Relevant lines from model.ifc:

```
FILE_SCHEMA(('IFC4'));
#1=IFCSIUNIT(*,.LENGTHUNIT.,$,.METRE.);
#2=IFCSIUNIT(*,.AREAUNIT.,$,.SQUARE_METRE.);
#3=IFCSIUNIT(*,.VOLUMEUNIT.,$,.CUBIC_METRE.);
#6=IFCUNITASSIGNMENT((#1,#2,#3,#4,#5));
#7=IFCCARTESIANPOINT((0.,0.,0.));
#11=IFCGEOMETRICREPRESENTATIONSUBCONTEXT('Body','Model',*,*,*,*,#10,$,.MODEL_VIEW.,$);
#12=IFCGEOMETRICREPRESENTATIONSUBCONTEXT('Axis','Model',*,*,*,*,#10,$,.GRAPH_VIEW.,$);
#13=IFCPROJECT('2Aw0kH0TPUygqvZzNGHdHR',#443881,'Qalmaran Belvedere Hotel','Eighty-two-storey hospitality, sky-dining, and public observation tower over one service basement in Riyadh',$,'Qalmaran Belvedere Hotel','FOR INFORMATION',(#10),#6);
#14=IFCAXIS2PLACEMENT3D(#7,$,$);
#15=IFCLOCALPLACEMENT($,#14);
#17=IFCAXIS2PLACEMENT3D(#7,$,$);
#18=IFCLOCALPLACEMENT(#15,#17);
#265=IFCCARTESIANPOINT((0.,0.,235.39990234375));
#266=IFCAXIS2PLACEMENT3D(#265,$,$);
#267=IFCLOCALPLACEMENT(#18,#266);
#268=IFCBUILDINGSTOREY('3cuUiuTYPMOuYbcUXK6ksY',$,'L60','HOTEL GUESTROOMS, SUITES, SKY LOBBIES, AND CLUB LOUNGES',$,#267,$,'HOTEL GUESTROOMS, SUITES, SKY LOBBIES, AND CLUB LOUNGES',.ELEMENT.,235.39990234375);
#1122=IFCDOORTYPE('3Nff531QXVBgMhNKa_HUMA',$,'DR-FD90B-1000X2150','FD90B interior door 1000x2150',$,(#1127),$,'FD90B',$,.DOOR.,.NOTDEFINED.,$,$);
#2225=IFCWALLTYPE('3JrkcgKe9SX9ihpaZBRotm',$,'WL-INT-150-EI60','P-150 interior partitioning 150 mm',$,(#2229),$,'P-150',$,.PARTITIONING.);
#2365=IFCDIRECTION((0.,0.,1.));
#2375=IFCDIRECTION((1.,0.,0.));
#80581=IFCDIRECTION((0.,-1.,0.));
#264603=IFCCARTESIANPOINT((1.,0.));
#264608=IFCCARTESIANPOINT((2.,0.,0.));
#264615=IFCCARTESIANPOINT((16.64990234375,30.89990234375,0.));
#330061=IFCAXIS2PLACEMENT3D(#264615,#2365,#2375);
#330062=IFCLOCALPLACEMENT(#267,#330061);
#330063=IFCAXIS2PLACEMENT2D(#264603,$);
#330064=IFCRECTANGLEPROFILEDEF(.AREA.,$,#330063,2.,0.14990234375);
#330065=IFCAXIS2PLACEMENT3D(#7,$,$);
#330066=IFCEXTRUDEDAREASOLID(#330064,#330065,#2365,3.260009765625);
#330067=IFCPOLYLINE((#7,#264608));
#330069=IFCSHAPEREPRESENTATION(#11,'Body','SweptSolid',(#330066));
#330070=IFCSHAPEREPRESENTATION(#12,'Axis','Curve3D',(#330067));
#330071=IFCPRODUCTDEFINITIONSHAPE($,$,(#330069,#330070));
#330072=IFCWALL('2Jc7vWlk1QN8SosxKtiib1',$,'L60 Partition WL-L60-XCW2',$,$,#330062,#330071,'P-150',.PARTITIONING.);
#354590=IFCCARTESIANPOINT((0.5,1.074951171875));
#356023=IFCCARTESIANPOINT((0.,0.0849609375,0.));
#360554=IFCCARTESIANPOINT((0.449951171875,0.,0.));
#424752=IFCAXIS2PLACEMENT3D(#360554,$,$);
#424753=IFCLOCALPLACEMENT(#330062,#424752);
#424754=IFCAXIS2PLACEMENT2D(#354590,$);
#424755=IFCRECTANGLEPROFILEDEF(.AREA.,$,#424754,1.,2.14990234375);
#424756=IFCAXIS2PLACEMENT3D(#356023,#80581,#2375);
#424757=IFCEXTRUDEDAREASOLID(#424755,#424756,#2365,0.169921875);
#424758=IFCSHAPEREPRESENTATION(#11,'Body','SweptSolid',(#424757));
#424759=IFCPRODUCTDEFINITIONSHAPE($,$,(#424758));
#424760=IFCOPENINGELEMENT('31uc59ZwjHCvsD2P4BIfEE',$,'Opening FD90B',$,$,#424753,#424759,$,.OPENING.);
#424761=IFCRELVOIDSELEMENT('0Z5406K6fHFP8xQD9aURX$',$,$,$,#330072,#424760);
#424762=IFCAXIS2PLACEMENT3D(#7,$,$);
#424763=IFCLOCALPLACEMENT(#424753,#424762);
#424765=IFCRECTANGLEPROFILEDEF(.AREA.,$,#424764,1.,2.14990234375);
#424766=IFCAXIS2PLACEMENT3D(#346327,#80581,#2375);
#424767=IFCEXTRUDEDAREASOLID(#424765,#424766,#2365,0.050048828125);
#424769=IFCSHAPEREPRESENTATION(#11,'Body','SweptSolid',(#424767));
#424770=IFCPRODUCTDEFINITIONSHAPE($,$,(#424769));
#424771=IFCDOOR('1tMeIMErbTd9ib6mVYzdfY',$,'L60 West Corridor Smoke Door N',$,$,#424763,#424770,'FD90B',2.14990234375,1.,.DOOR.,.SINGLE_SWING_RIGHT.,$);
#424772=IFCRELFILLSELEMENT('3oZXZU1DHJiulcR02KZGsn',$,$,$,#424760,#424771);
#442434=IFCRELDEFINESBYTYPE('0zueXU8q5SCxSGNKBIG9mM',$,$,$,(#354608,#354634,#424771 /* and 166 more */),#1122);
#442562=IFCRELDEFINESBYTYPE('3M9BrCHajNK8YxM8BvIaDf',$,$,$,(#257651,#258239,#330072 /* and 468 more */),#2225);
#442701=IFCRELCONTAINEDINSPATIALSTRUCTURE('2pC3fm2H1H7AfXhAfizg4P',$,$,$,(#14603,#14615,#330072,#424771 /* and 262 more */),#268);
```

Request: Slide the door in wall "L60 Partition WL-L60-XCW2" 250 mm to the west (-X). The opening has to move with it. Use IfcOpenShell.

```python
import ifcopenshell
import ifcopenshell.api.geometry
import ifcopenshell.util.placement
import ifcopenshell.util.unit

model = ifcopenshell.open("model.ifc")
unit_scale = ifcopenshell.util.unit.calculate_unit_scale(model)

door = model.by_guid("1tMeIMErbTd9ib6mVYzdfY")
opening = door.FillsVoids[0].RelatingOpeningElement
wall = opening.VoidsElements[0].RelatingBuildingElement

wall_matrix = ifcopenshell.util.placement.get_local_placement(wall.ObjectPlacement)
shift = wall_matrix[:3, 0] * -0.25 / unit_scale
before = ifcopenshell.util.placement.get_local_placement(door.ObjectPlacement)[:3, 3].copy()

# The door is placed relative to its opening, so it follows when the opening moves.
matrix = ifcopenshell.util.placement.get_local_placement(opening.ObjectPlacement)
matrix[:3, 3] += shift
ifcopenshell.api.geometry.edit_object_placement(
    model, product=opening, matrix=matrix, is_si=False, should_transform_children=True
)

after = ifcopenshell.util.placement.get_local_placement(door.ObjectPlacement)[:3, 3]
print("door moved by", (after - before).round(3) + 0.0)

model.write("model_rev.ifc")
```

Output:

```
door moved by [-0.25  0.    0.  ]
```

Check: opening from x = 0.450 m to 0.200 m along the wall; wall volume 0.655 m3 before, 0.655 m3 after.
